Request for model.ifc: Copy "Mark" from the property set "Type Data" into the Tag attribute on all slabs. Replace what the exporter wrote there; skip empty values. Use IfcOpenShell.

First a look at what the model holds.

```python
import ifcopenshell
import ifcopenshell.util.element

model = ifcopenshell.open("model.ifc")
print(model.schema)
slabs = model.by_type("IfcSlab")
print(len(slabs), "slabs")
for e in slabs[:8]:
    source = ifcopenshell.util.element.get_pset(e, "Type Data", "Mark")
    target = e.Tag
    print(e.id(), repr(source), repr(target), sep=" | ")
```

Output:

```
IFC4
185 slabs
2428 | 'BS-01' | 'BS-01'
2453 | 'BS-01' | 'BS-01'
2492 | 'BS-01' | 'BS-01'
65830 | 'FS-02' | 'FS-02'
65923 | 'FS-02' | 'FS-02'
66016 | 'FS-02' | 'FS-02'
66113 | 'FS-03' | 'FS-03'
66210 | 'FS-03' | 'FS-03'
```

```python
import ifcopenshell
import ifcopenshell.util.element

model = ifcopenshell.open("model.ifc")

count = 0
for e in model.by_type("IfcSlab"):
    value = ifcopenshell.util.element.get_pset(e, "Type Data", "Mark")
    current = e.Tag
    if not value or not value.strip() or current == value:
        continue
    e.Tag = value
    count += 1

print(count, "slabs updated")

model.write("model-out.ifc")
```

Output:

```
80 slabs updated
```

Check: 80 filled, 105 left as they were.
